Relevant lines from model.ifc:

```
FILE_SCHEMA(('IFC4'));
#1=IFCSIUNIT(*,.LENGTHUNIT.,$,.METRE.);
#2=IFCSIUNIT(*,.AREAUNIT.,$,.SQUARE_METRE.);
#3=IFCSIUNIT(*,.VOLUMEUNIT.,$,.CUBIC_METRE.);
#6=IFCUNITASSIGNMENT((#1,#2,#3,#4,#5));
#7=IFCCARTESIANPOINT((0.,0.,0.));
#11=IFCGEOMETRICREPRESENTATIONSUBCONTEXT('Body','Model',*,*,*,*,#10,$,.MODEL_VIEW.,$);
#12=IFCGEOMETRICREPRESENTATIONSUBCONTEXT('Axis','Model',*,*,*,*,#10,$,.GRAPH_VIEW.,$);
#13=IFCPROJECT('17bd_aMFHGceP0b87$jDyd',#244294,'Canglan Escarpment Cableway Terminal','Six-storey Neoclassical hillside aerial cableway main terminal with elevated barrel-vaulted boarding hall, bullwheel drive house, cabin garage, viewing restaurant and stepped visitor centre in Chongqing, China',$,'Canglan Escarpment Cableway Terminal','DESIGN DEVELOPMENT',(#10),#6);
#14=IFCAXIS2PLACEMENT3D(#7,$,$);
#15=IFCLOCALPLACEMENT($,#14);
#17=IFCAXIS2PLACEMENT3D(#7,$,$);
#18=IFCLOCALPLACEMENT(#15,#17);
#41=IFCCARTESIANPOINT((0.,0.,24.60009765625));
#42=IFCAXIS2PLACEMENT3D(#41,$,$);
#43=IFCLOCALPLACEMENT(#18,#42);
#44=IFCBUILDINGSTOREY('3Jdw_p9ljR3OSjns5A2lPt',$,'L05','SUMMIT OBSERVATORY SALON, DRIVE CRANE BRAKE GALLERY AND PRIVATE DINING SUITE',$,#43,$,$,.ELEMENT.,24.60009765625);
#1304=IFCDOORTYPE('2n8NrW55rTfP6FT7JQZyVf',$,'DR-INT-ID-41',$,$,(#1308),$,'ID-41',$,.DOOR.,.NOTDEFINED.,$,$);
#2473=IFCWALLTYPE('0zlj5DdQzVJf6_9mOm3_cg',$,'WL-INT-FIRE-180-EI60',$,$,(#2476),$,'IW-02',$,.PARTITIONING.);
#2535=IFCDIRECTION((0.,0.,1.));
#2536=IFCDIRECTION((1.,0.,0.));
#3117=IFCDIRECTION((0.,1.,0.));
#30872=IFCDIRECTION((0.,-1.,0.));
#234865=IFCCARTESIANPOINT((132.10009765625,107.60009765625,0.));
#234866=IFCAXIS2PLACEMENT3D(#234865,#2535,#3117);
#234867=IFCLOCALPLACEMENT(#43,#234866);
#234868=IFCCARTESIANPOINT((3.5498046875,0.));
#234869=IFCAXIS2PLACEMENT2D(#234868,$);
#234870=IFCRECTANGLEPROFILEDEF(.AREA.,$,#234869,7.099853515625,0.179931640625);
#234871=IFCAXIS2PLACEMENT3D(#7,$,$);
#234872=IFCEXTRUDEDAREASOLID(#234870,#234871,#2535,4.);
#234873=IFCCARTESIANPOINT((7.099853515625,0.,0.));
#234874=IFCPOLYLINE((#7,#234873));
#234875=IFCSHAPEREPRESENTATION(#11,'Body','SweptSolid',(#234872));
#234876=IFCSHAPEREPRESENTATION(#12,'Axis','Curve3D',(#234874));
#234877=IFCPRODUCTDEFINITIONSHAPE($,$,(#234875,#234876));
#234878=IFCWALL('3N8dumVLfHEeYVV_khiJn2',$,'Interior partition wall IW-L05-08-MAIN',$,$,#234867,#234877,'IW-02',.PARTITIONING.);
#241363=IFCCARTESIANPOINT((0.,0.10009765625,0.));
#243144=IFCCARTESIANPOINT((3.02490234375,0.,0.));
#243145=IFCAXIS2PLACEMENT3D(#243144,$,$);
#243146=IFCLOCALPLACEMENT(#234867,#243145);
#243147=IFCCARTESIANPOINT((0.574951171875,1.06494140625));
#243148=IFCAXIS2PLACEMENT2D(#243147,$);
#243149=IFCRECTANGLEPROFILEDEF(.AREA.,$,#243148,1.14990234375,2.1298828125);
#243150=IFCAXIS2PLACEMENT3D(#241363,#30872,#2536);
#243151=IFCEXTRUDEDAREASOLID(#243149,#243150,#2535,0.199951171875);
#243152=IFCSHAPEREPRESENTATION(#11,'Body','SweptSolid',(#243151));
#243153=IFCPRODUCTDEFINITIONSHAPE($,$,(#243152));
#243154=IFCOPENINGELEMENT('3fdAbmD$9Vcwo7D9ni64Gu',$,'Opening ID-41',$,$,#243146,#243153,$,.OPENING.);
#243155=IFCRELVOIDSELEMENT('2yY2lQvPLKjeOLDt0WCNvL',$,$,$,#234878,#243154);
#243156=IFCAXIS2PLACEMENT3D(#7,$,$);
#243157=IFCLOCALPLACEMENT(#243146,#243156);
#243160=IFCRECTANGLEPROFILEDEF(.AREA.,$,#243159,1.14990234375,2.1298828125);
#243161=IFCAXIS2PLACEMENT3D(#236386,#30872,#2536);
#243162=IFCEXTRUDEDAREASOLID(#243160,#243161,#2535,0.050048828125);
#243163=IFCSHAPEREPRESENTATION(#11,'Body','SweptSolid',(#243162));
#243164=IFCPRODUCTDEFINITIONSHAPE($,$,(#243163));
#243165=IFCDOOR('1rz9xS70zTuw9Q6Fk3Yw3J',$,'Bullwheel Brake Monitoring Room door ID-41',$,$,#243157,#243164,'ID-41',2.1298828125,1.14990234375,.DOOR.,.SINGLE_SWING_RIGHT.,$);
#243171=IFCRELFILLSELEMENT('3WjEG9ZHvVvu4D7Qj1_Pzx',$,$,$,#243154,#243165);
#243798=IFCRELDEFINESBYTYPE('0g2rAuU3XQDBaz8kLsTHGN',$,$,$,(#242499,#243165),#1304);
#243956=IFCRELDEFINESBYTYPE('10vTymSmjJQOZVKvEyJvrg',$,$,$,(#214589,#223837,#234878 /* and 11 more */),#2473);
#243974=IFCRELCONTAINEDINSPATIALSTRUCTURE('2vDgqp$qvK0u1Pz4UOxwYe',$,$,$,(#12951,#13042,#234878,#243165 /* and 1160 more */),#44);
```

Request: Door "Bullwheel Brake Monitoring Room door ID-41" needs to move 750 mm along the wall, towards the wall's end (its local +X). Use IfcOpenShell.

```python
import ifcopenshell
import ifcopenshell.api.geometry
import ifcopenshell.util.placement

model = ifcopenshell.open("model.ifc")

door = model.by_id(243165)
opening = door.FillsVoids[0].RelatingOpeningElement
wall = opening.VoidsElements[0].RelatingBuildingElement

wall_matrix = ifcopenshell.util.placement.get_local_placement(wall.ObjectPlacement)
shift = wall_matrix[:3, 0] * 0.75
before = ifcopenshell.util.placement.get_local_placement(door.ObjectPlacement)[:3, 3].copy()

# The door is placed relative to its opening, so it follows when the opening moves.
matrix = ifcopenshell.util.placement.get_local_placement(opening.ObjectPlacement)
matrix[:3, 3] += shift
ifcopenshell.api.geometry.edit_object_placement(
    model, product=opening, matrix=matrix, is_si=False, should_transform_children=True
)

after = ifcopenshell.util.placement.get_local_placement(door.ObjectPlacement)[:3, 3]
print("door moved by", (after - before).round(3) + 0.0)

model.write("model_edited.ifc")
```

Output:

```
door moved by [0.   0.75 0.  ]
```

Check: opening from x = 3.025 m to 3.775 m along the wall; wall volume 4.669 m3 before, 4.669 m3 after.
